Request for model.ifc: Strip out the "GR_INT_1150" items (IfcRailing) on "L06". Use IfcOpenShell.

First a look at what the model holds.

```python
import ifcopenshell
import ifcopenshell.util.element

model = ifcopenshell.open("model.ifc")
print(model.schema)
storey = next(s for s in model.by_type("IfcBuildingStorey") if s.Name == "L06")
railings = [e for e in ifcopenshell.util.element.get_decomposition(storey) if e.is_a("IfcRailing")]
seen = {}
for e in railings:
    element_type = ifcopenshell.util.element.get_type(e)
    name = element_type.Name if element_type not in (None, e) else None
    seen[name] = seen.get(name, 0) + 1
for name, count in sorted(seen.items(), key=str):
    print(count, "x", name)
```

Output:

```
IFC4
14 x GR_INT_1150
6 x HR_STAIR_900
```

```python
import ifcopenshell
import ifcopenshell.api.root
import ifcopenshell.util.element

model = ifcopenshell.open("model.ifc")

storey = next(s for s in model.by_type("IfcBuildingStorey") if s.Name == "L06")
railings = [e for e in ifcopenshell.util.element.get_decomposition(storey) if e.is_a("IfcRailing")]
targets = [e for e in railings if (t := ifcopenshell.util.element.get_type(e)) not in (None, e) and t.Name == "GR_INT_1150"]

for e in targets:
    ifcopenshell.api.root.remove_product(model, product=e)
print(len(targets), "removed")

model.write("model_v2.ifc")
```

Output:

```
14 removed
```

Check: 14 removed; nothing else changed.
